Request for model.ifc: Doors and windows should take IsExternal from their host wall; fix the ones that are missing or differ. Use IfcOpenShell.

First a look at what the model holds.

```python
import ifcopenshell
import ifcopenshell.util.element

model = ifcopenshell.open("model.ifc")
print(model.schema)
seen = {}
for e in model.by_type("IfcDoor") + model.by_type("IfcWindow"):
    if not e.FillsVoids:
        continue
    host = e.FillsVoids[0].RelatingOpeningElement.VoidsElements[0].RelatingBuildingElement
    own = ifcopenshell.util.element.get_pset(e, f"Pset_{e.is_a()[3:].removesuffix('StandardCase')}Common", "IsExternal")
    wall = ifcopenshell.util.element.get_pset(host, "Pset_WallCommon", "IsExternal")
    seen[e.is_a(), own, wall] = seen.get((e.is_a(), own, wall), 0) + 1
for (cls, own, wall), count in sorted(seen.items(), key=str):
    print(count, cls, "IsExternal:", own, "| host wall:", wall)
```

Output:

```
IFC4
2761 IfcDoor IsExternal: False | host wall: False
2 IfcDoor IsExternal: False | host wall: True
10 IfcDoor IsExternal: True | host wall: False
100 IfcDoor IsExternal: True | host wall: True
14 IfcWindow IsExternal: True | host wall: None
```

```python
import ifcopenshell
import ifcopenshell.api.pset
import ifcopenshell.util.element

model = ifcopenshell.open("model.ifc")

count = 0
for ifc_class, pset_name in (("IfcDoor", "Pset_DoorCommon"), ("IfcWindow", "Pset_WindowCommon")):
    for e in model.by_type(ifc_class):
        if not e.FillsVoids:
            continue
        host = e.FillsVoids[0].RelatingOpeningElement.VoidsElements[0].RelatingBuildingElement
        external = ifcopenshell.util.element.get_pset(host, "Pset_WallCommon", "IsExternal")
        if external is None or ifcopenshell.util.element.get_pset(e, pset_name, "IsExternal") == external:
            continue
        found = ifcopenshell.util.element.get_pset(e, pset_name, should_inherit=False)
        if found:
            pset = model.by_id(found["id"])
            if len(ifcopenshell.util.element.get_elements_by_pset(pset)) > 1:
                pset = ifcopenshell.api.pset.unshare_pset(model, products=[e], pset=pset)[0]
        else:
            pset = ifcopenshell.api.pset.add_pset(model, product=e, name=pset_name)
        ifcopenshell.api.pset.edit_pset(model, pset=pset, properties={"IsExternal": external})
        count += 1

print(count, "updated")

model.write("model_edited.ifc")
```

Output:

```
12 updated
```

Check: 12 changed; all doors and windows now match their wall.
